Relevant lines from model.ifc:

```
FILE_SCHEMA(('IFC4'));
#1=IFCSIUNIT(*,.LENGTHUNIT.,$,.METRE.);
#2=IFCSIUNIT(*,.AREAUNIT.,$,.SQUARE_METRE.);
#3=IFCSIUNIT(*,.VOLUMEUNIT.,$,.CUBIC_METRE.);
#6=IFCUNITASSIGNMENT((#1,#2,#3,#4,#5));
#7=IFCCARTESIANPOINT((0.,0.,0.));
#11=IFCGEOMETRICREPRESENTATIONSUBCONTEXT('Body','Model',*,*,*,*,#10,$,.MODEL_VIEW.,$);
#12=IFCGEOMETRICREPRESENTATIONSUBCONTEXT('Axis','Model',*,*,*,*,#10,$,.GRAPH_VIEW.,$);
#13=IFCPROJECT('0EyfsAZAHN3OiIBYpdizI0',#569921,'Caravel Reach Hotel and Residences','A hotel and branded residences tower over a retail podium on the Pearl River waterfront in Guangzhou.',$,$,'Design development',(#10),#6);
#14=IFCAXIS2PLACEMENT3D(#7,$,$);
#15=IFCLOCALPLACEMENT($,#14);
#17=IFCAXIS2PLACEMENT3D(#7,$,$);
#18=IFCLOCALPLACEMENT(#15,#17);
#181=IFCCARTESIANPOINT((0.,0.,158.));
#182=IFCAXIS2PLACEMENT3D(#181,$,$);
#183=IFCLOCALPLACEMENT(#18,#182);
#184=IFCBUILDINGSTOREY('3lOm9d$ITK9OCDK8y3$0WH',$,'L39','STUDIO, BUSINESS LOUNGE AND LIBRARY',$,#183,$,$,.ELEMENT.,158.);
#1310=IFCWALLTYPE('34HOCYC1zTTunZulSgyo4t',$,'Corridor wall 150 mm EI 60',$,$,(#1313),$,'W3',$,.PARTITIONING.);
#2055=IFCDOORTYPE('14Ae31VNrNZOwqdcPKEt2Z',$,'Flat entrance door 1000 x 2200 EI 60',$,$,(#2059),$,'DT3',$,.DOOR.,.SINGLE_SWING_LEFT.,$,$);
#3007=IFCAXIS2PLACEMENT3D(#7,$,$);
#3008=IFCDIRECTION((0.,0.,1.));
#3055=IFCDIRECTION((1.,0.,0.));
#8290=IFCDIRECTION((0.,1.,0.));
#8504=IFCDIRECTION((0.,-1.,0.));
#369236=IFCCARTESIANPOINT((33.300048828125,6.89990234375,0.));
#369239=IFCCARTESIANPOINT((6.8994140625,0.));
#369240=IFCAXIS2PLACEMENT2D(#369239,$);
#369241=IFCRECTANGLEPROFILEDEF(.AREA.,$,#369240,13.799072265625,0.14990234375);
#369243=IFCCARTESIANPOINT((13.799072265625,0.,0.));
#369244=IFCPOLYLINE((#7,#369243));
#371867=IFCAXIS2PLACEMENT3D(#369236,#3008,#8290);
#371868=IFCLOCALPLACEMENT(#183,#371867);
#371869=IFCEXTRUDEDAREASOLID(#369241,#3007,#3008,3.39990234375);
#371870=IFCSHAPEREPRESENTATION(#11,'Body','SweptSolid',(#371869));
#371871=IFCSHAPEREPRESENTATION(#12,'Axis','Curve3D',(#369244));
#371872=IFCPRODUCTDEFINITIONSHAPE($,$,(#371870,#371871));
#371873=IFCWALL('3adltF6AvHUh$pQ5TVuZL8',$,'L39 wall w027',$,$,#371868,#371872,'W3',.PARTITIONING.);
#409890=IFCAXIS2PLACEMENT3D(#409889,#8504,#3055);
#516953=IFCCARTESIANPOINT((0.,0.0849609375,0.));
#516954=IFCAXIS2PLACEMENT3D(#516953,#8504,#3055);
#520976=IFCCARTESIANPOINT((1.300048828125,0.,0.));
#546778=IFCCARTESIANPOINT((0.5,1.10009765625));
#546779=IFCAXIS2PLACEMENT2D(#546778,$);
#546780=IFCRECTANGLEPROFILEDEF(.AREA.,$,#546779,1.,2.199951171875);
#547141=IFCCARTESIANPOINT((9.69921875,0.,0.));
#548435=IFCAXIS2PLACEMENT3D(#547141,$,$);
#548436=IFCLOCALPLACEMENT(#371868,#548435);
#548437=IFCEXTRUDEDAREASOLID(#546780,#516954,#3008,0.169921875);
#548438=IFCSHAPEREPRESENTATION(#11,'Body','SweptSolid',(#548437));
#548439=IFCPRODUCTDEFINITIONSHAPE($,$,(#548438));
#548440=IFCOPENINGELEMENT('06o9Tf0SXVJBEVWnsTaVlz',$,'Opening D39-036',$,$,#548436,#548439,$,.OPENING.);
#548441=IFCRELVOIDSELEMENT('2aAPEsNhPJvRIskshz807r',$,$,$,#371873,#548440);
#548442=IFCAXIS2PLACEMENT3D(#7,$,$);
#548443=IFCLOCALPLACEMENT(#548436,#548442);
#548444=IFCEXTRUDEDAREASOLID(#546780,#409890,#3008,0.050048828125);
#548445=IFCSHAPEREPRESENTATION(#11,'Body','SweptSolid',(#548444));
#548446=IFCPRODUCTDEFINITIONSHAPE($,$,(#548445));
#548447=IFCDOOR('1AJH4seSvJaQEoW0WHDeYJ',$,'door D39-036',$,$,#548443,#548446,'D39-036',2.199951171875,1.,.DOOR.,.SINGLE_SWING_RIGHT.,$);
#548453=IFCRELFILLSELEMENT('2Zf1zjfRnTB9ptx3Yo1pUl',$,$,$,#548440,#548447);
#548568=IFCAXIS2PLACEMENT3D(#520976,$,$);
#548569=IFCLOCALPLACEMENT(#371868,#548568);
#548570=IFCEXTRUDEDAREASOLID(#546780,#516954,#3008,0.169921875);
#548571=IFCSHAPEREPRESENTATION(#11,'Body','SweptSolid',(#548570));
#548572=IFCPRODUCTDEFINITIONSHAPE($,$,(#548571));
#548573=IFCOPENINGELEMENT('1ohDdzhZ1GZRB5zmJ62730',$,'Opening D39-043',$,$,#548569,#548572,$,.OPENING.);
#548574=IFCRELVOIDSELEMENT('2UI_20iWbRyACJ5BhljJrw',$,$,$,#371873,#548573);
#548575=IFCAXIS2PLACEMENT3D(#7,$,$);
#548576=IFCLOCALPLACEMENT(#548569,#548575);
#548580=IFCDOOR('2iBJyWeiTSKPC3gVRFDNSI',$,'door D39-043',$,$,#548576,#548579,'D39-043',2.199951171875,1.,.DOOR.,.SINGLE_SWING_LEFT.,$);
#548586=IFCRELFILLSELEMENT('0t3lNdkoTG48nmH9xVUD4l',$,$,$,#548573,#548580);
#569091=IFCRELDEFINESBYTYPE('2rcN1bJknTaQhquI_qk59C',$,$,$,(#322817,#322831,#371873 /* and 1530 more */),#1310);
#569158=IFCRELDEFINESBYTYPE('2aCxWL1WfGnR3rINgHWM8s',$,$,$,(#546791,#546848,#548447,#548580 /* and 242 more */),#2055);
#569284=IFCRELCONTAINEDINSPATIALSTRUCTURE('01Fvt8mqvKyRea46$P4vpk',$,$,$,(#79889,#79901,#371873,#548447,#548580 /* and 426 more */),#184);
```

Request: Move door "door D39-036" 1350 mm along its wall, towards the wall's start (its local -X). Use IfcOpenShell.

```python
import ifcopenshell
import ifcopenshell.api.geometry
import ifcopenshell.util.placement

model = ifcopenshell.open("model.ifc")

door = model.by_guid("1AJH4seSvJaQEoW0WHDeYJ")
opening = door.FillsVoids[0].RelatingOpeningElement
wall = opening.VoidsElements[0].RelatingBuildingElement

wall_matrix = ifcopenshell.util.placement.get_local_placement(wall.ObjectPlacement)
shift = wall_matrix[:3, 0] * -1.35
before = ifcopenshell.util.placement.get_local_placement(door.ObjectPlacement)[:3, 3].copy()

# The door is placed relative to its opening, so it follows when the opening moves.
matrix = ifcopenshell.util.placement.get_local_placement(opening.ObjectPlacement)
matrix[:3, 3] += shift
ifcopenshell.api.geometry.edit_object_placement(
    model, product=opening, matrix=matrix, is_si=False, should_transform_children=True
)

after = ifcopenshell.util.placement.get_local_placement(door.ObjectPlacement)[:3, 3]
print("door moved by", (after - before).round(3) + 0.0)

model.write("model-out.ifc")
```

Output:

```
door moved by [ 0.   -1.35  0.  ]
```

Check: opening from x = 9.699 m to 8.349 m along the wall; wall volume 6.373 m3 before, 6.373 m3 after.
